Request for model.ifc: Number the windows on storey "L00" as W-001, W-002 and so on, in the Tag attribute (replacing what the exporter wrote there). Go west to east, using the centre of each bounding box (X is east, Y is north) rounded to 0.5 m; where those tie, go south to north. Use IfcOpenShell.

First a look at what the model holds.

```python
import ifcopenshell
import ifcopenshell.util.element
import ifcopenshell.util.placement

model = ifcopenshell.open("model.ifc")
print(model.schema)
storey = next(s for s in model.by_type("IfcBuildingStorey") if s.Name == "L00")
windows = [e for e in ifcopenshell.util.element.get_decomposition(storey) if e.is_a("IfcWindow")]
for e in sorted(windows, key=lambda e: e.id()):
    origin = ifcopenshell.util.placement.get_local_placement(e.ObjectPlacement)[:3, 3]
    print(e.id(), e.Tag, e.Name, origin.round(2) + 0.0, sep=" | ")
```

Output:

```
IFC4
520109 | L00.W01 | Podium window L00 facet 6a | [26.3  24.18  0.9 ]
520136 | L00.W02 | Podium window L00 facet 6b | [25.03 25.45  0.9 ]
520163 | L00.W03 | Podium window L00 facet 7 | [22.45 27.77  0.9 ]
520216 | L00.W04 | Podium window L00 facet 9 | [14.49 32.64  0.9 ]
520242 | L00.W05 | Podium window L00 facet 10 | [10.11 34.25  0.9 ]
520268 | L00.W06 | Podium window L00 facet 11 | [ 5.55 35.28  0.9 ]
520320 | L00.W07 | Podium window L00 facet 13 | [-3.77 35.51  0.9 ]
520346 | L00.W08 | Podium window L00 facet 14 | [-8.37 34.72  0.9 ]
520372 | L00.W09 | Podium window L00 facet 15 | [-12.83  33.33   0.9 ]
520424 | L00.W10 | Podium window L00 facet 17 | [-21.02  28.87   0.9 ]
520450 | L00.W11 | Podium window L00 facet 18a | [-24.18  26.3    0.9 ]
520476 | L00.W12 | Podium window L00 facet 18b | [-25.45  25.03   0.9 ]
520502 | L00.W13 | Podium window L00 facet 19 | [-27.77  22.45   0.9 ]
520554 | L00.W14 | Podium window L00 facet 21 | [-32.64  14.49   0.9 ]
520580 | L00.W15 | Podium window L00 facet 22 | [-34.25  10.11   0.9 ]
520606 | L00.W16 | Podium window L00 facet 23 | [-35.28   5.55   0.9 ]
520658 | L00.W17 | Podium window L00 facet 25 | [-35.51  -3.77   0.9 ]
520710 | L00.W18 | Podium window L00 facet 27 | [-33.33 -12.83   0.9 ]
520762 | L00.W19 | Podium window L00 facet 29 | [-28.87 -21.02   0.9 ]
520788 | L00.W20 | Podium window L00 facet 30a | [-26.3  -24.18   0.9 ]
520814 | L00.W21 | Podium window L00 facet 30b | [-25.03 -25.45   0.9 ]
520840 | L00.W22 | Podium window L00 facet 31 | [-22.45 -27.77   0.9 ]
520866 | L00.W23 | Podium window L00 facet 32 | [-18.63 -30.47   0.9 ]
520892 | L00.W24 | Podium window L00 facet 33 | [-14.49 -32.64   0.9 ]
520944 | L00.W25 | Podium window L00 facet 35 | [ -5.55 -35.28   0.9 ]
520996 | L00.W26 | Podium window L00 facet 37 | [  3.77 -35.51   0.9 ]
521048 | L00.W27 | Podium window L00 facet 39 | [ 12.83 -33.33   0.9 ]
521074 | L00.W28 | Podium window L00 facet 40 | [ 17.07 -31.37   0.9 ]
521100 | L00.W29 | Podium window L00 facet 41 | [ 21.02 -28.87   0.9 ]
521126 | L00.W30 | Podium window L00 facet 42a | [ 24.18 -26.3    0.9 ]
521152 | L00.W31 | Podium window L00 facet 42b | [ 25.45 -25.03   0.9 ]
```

```python
import ifcopenshell
import ifcopenshell.geom
import ifcopenshell.util.element
import ifcopenshell.util.shape

model = ifcopenshell.open("model.ifc")
settings = ifcopenshell.geom.settings()
settings.set("use-world-coords", True)


def centre(element):
    shape = ifcopenshell.geom.create_shape(settings, element)
    return ifcopenshell.util.shape.get_bbox_centroid(shape.geometry)


storey = next(s for s in model.by_type("IfcBuildingStorey") if s.Name == "L00")
windows = [e for e in ifcopenshell.util.element.get_decomposition(storey) if e.is_a("IfcWindow")]

# Insertion points can sit at a corner or the storey origin, so sort by the geometry (in metres).
centres = {e: centre(e) for e in windows}
windows.sort(key=lambda e: (round(centres[e][0] / 0.5), centres[e][1]))

for i, e in enumerate(windows, start=1):
    number = f"W-0{i:02d}"
    e.Tag = number
    print(e.id(), number)

model.write("model-out.ifc")
```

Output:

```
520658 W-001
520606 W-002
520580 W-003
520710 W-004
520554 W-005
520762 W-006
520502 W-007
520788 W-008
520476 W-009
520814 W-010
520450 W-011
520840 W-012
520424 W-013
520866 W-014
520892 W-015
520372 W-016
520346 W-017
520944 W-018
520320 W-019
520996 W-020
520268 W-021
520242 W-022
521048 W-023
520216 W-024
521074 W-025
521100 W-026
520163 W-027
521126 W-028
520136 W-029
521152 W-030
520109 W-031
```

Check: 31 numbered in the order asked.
